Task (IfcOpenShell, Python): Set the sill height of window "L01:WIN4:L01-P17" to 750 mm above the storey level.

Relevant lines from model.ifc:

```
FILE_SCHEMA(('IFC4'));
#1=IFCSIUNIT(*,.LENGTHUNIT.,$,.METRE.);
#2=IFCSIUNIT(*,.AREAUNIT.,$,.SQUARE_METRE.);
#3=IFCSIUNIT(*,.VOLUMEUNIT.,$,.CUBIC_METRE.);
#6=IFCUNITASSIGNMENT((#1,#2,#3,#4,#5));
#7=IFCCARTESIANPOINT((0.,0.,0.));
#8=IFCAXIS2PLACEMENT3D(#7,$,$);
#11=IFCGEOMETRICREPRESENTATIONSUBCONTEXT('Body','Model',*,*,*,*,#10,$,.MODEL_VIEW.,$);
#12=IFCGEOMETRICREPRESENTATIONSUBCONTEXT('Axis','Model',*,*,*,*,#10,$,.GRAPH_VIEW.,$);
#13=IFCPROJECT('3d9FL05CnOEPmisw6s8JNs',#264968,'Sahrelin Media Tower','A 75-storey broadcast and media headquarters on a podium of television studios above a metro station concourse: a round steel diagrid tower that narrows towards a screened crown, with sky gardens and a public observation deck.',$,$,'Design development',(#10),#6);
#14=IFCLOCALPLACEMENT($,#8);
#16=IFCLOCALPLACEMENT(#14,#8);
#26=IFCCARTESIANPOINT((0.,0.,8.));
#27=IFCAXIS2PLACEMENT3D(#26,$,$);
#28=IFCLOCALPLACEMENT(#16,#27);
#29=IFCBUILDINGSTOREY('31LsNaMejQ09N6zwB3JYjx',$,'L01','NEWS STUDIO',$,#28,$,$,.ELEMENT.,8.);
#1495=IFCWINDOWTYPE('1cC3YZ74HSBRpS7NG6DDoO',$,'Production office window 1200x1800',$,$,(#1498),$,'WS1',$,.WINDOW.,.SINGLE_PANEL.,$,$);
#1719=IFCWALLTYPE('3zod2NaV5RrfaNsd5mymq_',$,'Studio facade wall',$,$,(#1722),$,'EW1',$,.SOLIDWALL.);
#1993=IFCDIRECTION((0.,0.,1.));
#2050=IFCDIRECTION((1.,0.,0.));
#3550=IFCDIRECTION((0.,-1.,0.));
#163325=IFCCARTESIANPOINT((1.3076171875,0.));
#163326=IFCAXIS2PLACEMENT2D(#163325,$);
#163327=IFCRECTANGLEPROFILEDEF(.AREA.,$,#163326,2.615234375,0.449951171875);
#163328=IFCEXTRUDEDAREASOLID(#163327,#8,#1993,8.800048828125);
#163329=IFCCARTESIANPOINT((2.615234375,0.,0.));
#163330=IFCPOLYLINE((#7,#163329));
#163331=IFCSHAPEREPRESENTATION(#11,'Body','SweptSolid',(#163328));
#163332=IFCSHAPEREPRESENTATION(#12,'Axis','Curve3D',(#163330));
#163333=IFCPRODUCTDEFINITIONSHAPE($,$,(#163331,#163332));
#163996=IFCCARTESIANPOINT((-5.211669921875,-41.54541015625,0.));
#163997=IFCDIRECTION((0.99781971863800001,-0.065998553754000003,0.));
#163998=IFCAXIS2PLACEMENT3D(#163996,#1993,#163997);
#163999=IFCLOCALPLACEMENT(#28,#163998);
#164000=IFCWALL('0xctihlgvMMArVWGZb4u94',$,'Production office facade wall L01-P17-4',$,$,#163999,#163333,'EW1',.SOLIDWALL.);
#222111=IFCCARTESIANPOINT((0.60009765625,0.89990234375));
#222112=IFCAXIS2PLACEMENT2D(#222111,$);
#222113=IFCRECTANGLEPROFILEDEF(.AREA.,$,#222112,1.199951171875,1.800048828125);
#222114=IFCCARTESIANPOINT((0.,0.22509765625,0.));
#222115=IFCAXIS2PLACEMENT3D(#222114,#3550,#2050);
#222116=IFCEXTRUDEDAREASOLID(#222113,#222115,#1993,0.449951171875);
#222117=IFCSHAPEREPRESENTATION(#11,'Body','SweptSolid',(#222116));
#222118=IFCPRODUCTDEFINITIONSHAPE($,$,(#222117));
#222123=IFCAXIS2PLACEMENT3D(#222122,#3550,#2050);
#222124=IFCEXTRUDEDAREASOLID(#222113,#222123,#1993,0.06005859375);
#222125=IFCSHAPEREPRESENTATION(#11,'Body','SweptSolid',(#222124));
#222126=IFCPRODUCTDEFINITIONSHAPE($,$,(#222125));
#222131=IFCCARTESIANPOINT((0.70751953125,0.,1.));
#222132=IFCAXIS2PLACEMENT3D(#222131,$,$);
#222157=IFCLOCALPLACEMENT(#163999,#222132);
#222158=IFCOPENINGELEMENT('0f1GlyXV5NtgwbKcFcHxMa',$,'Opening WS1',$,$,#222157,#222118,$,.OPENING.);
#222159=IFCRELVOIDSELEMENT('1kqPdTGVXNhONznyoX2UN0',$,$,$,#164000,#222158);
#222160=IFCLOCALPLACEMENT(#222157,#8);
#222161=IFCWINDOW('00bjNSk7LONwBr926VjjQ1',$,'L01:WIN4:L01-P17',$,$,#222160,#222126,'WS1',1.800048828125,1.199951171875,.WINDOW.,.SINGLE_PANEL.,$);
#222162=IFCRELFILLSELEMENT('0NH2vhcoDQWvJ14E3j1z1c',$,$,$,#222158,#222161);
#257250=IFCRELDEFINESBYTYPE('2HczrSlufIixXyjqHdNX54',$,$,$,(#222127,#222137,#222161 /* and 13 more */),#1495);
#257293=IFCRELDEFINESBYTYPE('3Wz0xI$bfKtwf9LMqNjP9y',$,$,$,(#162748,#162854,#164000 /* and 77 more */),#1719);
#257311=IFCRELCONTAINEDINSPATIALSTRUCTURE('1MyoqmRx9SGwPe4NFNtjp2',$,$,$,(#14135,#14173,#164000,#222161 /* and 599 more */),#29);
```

```python
import numpy as np
import ifcopenshell
import ifcopenshell.api.geometry
import ifcopenshell.geom
import ifcopenshell.util.element
import ifcopenshell.util.placement
import ifcopenshell.util.shape
import ifcopenshell.util.unit

model = ifcopenshell.open("model.ifc")
unit_scale = ifcopenshell.util.unit.calculate_unit_scale(model)

window = model.by_guid("00bjNSk7LONwBr926VjjQ1")
opening = window.FillsVoids[0].RelatingOpeningElement
storey = ifcopenshell.util.element.get_container(window, ifc_class="IfcBuildingStorey")
level = ifcopenshell.util.placement.get_local_placement(storey.ObjectPlacement)[2, 3]

# The opening's origin need not be at the sill, so measure its lowest point.
shape = ifcopenshell.geom.create_shape(ifcopenshell.geom.settings(), opening)
bottom = ifcopenshell.util.shape.get_shape_bottom_elevation(shape, shape.geometry) / unit_scale
dz = level + 0.75 / unit_scale - bottom

shift = np.array([0.0, 0.0, dz])
# The window is placed relative to its opening, so it follows when the opening moves.
matrix = ifcopenshell.util.placement.get_local_placement(opening.ObjectPlacement)
matrix[:3, 3] += shift
ifcopenshell.api.geometry.edit_object_placement(
    model, product=opening, matrix=matrix, is_si=False, should_transform_children=True
)

print(f"moved by {dz * unit_scale:+.3f} m")

model.write("model_rev.ifc")
```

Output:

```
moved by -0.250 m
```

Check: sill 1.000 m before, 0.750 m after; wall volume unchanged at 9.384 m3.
